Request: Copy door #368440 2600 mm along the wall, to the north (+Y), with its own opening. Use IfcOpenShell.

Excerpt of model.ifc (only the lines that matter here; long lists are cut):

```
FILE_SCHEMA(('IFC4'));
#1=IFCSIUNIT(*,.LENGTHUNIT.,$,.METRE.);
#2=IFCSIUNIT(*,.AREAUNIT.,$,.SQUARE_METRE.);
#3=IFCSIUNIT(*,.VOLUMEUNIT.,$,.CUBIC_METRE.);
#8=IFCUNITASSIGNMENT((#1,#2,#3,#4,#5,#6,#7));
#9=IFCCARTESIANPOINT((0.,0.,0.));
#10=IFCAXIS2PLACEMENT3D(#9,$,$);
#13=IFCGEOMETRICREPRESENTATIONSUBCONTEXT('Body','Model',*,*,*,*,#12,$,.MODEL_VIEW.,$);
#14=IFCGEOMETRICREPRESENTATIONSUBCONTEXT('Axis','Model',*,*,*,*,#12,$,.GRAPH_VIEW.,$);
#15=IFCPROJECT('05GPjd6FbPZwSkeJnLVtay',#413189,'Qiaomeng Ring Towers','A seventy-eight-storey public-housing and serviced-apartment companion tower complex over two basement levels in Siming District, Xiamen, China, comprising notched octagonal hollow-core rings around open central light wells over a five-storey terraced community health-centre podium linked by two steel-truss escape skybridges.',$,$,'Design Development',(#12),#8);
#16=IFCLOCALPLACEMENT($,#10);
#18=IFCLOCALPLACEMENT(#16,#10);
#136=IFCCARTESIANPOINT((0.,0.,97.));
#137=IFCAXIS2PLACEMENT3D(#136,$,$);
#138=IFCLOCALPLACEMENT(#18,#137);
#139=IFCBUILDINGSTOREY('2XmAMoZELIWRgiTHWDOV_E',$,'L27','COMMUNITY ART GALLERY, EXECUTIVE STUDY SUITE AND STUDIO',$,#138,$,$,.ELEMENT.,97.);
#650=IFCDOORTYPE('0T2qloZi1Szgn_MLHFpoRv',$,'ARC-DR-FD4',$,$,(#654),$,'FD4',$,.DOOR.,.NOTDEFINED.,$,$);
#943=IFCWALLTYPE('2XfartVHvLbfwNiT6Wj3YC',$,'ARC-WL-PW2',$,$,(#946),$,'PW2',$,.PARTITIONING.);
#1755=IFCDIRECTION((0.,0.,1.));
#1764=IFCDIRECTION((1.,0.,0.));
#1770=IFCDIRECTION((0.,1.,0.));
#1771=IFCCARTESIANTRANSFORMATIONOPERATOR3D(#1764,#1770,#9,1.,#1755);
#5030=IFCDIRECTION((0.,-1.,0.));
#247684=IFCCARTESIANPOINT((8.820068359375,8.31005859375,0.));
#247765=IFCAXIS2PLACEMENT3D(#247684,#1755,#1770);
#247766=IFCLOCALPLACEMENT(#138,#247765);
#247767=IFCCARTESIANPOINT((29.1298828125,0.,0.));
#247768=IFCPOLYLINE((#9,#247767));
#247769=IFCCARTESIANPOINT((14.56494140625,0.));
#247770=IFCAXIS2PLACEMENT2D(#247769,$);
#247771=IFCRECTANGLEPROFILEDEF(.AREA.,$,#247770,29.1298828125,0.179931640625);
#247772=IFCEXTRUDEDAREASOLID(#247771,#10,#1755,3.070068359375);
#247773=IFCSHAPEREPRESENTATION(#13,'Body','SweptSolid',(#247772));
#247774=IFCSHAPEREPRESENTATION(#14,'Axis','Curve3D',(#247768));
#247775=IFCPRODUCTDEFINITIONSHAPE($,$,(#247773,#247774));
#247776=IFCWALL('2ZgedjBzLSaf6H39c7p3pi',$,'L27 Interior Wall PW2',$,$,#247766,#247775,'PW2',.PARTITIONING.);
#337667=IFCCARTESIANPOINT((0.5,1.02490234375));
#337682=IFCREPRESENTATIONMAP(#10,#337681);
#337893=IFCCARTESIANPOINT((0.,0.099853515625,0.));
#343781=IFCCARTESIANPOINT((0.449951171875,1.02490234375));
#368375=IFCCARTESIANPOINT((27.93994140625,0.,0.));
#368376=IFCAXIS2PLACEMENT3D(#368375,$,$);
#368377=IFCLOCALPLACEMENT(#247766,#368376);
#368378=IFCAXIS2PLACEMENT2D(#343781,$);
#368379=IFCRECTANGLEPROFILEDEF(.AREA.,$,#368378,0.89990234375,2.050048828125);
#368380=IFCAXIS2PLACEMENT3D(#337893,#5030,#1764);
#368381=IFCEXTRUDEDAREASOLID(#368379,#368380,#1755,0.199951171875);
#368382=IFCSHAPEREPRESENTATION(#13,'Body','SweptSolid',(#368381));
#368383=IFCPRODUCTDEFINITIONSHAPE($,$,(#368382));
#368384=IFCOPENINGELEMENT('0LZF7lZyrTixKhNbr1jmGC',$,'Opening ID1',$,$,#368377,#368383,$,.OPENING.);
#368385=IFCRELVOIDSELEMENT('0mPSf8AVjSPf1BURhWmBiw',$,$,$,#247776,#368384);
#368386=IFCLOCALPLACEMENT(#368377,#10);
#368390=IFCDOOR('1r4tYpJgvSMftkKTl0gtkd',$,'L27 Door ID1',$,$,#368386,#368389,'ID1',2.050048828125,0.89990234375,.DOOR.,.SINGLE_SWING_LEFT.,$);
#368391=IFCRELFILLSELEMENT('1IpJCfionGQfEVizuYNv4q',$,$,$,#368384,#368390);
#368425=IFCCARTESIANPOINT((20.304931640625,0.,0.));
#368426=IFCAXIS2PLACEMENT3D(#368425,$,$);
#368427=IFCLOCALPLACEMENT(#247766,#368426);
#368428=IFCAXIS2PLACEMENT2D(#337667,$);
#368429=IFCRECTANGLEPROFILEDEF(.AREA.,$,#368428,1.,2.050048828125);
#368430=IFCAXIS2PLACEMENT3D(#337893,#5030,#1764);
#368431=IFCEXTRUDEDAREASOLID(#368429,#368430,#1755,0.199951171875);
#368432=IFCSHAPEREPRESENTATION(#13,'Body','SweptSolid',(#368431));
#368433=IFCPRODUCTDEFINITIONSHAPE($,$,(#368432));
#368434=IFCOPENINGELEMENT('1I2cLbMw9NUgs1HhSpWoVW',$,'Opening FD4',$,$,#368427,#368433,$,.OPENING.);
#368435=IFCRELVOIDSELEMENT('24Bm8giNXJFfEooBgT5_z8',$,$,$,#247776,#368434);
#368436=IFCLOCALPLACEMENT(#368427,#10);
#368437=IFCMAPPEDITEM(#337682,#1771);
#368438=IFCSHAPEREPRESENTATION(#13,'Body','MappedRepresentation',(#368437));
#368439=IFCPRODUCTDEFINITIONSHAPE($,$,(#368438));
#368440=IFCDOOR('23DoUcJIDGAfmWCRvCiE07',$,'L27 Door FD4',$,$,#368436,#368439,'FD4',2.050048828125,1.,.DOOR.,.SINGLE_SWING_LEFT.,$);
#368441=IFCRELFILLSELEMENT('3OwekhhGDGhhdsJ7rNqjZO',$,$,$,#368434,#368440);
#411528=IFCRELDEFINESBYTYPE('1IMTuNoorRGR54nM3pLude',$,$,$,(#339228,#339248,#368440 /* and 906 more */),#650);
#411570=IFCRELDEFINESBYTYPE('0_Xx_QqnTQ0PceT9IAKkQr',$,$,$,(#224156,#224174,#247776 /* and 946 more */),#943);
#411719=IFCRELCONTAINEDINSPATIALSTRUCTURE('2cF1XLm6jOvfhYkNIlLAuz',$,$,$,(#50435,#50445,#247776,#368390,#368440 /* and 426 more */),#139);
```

```python
import ifcopenshell
import ifcopenshell.api.feature
import ifcopenshell.api.geometry
import ifcopenshell.api.root
import ifcopenshell.geom
import ifcopenshell.util.element
import ifcopenshell.util.placement
import ifcopenshell.util.shape
import ifcopenshell.util.unit

model = ifcopenshell.open("model.ifc")
unit_scale = ifcopenshell.util.unit.calculate_unit_scale(model)
settings = ifcopenshell.geom.settings()


def volume(element):
    """Net volume in cubic metres, openings subtracted."""
    shape = ifcopenshell.geom.create_shape(settings, element)
    return ifcopenshell.util.shape.get_volume(shape.geometry)


door = model.by_id(368440)
opening = door.FillsVoids[0].RelatingOpeningElement
wall = opening.VoidsElements[0].RelatingBuildingElement
before = volume(wall)
shift = ifcopenshell.util.placement.get_local_placement(wall.ObjectPlacement)[:3, 0] * 2.6 / unit_scale

# copy_class copies the void relationship, type, container and properties, but no geometry.
new_opening = ifcopenshell.api.root.copy_class(model, product=opening)
new_opening.Representation = ifcopenshell.util.element.copy_deep(
    model, opening.Representation, exclude=["IfcGeometricRepresentationContext", "IfcRepresentationMap"]
)
new_door = ifcopenshell.api.root.copy_class(model, product=door)
new_door.Representation = ifcopenshell.util.element.copy_deep(
    model, door.Representation, exclude=["IfcGeometricRepresentationContext", "IfcRepresentationMap"]
)
new_door.Tag = None
ifcopenshell.api.feature.add_filling(model, opening=new_opening, element=new_door)

for old, new in ((opening, new_opening), (door, new_door)):
    matrix = ifcopenshell.util.placement.get_local_placement(old.ObjectPlacement)
    matrix[:3, 3] += shift
    ifcopenshell.api.geometry.edit_object_placement(model, product=new, matrix=matrix, is_si=False)

after = volume(wall)

print(f"wall volume {before:.3f} -> {after:.3f} m3")

model.write("model_updated.ifc")
```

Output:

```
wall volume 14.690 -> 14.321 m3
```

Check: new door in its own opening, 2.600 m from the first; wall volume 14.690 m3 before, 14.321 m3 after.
